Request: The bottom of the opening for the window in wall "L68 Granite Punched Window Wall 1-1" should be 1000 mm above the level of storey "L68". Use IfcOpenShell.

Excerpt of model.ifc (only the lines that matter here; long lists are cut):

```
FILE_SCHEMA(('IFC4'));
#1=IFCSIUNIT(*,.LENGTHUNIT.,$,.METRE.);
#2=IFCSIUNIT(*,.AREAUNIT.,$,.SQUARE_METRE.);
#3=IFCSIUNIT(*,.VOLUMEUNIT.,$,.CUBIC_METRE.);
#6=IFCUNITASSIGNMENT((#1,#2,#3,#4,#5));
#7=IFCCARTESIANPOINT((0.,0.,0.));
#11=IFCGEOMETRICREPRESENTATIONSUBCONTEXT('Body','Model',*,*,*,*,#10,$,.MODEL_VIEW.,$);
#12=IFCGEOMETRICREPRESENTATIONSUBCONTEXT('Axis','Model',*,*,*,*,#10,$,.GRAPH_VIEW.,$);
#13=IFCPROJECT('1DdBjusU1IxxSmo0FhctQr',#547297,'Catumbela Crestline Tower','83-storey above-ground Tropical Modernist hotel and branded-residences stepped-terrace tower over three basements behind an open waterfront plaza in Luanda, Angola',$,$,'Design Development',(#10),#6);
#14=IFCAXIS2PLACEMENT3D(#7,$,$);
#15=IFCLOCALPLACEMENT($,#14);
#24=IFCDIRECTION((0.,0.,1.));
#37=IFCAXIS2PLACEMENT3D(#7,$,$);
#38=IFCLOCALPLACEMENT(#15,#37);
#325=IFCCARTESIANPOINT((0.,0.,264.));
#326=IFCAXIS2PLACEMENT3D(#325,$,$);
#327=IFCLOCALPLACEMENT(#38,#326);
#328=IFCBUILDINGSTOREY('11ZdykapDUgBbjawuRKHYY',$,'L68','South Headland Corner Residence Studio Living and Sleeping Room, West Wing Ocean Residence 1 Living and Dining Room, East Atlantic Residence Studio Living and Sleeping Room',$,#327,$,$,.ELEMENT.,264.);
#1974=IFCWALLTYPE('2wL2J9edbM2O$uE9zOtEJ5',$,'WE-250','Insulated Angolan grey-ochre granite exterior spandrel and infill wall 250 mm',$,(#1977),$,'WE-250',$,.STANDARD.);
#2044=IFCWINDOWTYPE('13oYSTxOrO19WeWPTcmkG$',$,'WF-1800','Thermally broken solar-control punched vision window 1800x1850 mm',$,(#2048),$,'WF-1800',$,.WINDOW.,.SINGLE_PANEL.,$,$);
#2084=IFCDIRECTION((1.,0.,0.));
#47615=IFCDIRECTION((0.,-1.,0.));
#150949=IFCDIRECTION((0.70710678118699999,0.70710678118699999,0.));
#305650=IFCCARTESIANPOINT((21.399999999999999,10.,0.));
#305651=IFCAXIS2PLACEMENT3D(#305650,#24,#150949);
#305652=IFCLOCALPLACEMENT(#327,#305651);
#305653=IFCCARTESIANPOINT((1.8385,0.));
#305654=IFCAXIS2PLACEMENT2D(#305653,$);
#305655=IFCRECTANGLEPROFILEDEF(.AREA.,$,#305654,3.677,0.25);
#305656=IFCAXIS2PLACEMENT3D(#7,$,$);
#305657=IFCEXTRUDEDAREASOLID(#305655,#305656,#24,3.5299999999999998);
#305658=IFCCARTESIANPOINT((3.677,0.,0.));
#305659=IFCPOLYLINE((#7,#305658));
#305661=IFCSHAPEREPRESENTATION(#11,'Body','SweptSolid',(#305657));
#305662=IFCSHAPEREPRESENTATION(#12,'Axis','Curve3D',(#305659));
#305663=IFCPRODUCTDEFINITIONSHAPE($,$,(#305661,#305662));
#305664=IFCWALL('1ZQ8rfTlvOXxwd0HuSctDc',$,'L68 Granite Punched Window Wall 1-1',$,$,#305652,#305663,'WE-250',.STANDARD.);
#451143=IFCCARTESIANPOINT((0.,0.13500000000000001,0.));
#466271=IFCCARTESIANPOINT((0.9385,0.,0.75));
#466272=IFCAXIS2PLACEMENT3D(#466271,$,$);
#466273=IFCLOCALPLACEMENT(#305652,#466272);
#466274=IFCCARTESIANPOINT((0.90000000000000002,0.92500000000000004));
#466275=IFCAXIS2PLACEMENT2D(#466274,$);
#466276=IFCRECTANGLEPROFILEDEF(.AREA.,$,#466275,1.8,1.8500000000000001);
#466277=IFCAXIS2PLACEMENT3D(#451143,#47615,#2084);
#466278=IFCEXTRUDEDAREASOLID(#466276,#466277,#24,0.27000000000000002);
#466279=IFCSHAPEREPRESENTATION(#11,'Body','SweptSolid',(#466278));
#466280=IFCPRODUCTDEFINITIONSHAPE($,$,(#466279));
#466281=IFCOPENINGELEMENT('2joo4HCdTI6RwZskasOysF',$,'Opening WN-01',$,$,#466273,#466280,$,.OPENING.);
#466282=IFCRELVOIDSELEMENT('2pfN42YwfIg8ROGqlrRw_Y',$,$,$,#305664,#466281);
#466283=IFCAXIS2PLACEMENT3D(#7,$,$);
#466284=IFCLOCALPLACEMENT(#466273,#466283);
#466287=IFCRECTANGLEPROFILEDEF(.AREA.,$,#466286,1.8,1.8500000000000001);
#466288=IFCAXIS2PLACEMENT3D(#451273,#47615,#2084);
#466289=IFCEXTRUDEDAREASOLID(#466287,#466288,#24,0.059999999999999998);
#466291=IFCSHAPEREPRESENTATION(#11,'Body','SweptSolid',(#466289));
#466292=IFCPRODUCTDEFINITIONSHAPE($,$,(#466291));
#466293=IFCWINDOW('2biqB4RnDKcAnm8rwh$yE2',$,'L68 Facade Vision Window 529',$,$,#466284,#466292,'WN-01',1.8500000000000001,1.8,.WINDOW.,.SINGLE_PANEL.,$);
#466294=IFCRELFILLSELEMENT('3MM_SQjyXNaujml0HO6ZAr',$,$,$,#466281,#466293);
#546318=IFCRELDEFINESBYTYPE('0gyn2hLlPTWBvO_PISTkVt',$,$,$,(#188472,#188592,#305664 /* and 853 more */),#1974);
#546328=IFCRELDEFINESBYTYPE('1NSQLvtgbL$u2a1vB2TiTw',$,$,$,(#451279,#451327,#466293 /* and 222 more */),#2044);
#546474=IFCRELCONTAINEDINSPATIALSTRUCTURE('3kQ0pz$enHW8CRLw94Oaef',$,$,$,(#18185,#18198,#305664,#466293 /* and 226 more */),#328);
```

```python
import numpy as np
import ifcopenshell
import ifcopenshell.api.geometry
import ifcopenshell.geom
import ifcopenshell.util.element
import ifcopenshell.util.placement
import ifcopenshell.util.shape
import ifcopenshell.util.unit

model = ifcopenshell.open("model.ifc")
unit_scale = ifcopenshell.util.unit.calculate_unit_scale(model)

window = model.by_guid("2biqB4RnDKcAnm8rwh$yE2")
opening = window.FillsVoids[0].RelatingOpeningElement
storey = ifcopenshell.util.element.get_container(window, ifc_class="IfcBuildingStorey")
level = ifcopenshell.util.placement.get_local_placement(storey.ObjectPlacement)[2, 3]

# The opening's origin need not be at the sill, so measure its lowest point.
shape = ifcopenshell.geom.create_shape(ifcopenshell.geom.settings(), opening)
bottom = ifcopenshell.util.shape.get_shape_bottom_elevation(shape, shape.geometry) / unit_scale
dz = level + 1.0 - bottom

shift = np.array([0.0, 0.0, dz])
# The window is placed relative to its opening, so it follows when the opening moves.
matrix = ifcopenshell.util.placement.get_local_placement(opening.ObjectPlacement)
matrix[:3, 3] += shift
ifcopenshell.api.geometry.edit_object_placement(
    model, product=opening, matrix=matrix, is_si=False, should_transform_children=True
)

print(f"moved by {dz * unit_scale:+.3f} m")

model.write("model_rev.ifc")
```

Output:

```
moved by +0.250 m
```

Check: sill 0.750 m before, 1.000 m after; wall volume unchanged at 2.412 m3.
